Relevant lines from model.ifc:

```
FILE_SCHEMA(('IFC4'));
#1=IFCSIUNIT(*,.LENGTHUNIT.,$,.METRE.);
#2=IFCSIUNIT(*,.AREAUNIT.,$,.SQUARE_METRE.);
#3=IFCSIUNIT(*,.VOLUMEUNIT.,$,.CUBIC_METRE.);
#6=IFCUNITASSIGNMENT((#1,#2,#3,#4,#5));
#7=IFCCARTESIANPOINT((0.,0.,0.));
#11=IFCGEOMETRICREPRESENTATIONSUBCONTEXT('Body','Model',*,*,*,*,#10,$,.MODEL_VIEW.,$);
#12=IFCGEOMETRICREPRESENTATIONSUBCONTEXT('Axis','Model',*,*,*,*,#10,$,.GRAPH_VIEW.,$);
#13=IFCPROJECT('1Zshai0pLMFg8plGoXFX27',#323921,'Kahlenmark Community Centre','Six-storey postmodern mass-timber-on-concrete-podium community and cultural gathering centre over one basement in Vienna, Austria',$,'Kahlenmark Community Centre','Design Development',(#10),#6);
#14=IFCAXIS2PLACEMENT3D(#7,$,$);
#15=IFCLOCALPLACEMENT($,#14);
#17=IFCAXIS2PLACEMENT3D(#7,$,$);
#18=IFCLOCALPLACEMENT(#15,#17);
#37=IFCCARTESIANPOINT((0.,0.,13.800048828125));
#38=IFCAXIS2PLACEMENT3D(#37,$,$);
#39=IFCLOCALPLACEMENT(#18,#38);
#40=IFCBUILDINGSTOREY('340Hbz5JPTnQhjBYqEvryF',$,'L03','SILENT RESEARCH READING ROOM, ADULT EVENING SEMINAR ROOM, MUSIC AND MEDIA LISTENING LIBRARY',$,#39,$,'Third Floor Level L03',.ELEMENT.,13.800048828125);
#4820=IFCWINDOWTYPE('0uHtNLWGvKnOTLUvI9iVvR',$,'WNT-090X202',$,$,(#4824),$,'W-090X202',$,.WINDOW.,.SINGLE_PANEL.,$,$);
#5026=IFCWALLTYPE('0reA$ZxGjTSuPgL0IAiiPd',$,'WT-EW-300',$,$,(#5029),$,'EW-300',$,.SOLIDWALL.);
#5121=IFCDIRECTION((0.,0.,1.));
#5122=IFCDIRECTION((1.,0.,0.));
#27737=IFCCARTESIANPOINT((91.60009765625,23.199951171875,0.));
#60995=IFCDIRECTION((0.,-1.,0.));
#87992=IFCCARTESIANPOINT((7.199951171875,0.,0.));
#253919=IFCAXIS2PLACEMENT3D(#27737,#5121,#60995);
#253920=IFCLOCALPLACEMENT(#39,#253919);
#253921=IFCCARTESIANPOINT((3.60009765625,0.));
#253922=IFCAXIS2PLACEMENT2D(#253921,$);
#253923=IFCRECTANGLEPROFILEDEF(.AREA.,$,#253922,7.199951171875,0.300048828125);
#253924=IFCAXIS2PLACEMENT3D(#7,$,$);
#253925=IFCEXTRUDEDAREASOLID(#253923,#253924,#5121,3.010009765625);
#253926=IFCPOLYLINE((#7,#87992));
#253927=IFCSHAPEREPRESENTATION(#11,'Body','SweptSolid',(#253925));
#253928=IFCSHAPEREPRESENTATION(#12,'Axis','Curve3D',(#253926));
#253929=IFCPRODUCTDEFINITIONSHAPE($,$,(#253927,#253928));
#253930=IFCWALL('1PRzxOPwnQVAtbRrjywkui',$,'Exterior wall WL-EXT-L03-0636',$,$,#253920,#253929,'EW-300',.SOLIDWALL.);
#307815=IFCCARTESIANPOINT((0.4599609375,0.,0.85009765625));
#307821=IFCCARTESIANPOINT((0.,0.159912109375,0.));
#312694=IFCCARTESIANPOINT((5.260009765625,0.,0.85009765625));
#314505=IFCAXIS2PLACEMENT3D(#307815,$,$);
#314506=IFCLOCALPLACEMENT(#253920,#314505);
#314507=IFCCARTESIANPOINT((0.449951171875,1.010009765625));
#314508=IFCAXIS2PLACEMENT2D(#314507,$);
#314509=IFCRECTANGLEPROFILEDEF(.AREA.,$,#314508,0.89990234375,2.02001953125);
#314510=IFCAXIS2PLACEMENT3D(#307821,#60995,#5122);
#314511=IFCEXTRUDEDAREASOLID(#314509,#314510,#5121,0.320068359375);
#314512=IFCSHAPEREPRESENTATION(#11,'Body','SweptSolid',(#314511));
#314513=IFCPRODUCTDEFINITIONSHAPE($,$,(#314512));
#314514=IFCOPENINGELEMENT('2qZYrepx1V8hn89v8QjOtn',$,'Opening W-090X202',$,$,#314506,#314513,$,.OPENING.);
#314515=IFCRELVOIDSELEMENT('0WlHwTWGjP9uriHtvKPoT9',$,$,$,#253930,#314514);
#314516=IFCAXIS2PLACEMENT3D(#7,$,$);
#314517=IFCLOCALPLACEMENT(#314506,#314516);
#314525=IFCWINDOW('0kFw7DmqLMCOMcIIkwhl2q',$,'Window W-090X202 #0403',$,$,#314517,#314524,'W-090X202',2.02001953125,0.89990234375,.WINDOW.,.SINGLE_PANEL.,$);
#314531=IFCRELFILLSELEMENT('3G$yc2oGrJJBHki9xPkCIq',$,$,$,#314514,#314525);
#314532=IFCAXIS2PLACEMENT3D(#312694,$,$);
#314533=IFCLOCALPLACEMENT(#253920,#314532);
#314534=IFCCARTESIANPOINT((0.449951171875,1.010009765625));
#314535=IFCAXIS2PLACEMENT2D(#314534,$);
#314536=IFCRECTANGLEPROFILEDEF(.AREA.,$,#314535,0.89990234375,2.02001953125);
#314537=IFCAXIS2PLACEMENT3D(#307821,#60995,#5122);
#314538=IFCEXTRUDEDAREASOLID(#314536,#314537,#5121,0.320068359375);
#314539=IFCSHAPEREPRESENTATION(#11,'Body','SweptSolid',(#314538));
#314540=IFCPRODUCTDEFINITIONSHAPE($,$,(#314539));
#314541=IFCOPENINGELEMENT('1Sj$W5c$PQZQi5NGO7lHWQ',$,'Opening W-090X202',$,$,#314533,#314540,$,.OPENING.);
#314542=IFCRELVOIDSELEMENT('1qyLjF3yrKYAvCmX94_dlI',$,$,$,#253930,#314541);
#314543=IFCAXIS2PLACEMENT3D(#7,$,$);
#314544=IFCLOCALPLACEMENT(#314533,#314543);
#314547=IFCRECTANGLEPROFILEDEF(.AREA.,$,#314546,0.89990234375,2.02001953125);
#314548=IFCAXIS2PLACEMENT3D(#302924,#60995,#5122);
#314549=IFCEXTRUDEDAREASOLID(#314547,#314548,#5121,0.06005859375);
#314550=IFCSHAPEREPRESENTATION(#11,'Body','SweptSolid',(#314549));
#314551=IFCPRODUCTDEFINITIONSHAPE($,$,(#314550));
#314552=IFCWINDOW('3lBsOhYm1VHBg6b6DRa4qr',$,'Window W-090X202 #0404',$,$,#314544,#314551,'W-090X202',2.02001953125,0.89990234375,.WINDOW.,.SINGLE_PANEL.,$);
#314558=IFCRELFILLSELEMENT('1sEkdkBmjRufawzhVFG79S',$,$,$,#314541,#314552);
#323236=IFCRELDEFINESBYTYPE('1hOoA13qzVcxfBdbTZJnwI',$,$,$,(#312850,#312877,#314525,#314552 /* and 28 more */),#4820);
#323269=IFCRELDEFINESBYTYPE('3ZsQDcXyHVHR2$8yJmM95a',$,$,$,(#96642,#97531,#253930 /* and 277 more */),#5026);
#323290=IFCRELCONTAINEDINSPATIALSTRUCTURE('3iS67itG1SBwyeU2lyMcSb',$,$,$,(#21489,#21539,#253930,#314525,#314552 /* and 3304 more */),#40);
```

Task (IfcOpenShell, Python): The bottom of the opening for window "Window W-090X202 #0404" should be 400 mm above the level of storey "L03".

```python
import numpy as np
import ifcopenshell
import ifcopenshell.api.geometry
import ifcopenshell.geom
import ifcopenshell.util.element
import ifcopenshell.util.placement
import ifcopenshell.util.shape
import ifcopenshell.util.unit

model = ifcopenshell.open("model.ifc")
unit_scale = ifcopenshell.util.unit.calculate_unit_scale(model)

window = model.by_id(314552)
opening = window.FillsVoids[0].RelatingOpeningElement
storey = ifcopenshell.util.element.get_container(window, ifc_class="IfcBuildingStorey")
level = ifcopenshell.util.placement.get_local_placement(storey.ObjectPlacement)[2, 3]

# The opening's origin need not be at the sill, so measure its lowest point.
shape = ifcopenshell.geom.create_shape(ifcopenshell.geom.settings(), opening)
bottom = ifcopenshell.util.shape.get_shape_bottom_elevation(shape, shape.geometry) / unit_scale
dz = level + 0.4 - bottom

shift = np.array([0.0, 0.0, dz])
# The window is placed relative to its opening, so it follows when the opening moves.
matrix = ifcopenshell.util.placement.get_local_placement(opening.ObjectPlacement)
matrix[:3, 3] += shift
ifcopenshell.api.geometry.edit_object_placement(
    model, product=opening, matrix=matrix, is_si=False, should_transform_children=True
)

print(f"moved by {dz * unit_scale:+.3f} m")

model.write("model-out.ifc")
```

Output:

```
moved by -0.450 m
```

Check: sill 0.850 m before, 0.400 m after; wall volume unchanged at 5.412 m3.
